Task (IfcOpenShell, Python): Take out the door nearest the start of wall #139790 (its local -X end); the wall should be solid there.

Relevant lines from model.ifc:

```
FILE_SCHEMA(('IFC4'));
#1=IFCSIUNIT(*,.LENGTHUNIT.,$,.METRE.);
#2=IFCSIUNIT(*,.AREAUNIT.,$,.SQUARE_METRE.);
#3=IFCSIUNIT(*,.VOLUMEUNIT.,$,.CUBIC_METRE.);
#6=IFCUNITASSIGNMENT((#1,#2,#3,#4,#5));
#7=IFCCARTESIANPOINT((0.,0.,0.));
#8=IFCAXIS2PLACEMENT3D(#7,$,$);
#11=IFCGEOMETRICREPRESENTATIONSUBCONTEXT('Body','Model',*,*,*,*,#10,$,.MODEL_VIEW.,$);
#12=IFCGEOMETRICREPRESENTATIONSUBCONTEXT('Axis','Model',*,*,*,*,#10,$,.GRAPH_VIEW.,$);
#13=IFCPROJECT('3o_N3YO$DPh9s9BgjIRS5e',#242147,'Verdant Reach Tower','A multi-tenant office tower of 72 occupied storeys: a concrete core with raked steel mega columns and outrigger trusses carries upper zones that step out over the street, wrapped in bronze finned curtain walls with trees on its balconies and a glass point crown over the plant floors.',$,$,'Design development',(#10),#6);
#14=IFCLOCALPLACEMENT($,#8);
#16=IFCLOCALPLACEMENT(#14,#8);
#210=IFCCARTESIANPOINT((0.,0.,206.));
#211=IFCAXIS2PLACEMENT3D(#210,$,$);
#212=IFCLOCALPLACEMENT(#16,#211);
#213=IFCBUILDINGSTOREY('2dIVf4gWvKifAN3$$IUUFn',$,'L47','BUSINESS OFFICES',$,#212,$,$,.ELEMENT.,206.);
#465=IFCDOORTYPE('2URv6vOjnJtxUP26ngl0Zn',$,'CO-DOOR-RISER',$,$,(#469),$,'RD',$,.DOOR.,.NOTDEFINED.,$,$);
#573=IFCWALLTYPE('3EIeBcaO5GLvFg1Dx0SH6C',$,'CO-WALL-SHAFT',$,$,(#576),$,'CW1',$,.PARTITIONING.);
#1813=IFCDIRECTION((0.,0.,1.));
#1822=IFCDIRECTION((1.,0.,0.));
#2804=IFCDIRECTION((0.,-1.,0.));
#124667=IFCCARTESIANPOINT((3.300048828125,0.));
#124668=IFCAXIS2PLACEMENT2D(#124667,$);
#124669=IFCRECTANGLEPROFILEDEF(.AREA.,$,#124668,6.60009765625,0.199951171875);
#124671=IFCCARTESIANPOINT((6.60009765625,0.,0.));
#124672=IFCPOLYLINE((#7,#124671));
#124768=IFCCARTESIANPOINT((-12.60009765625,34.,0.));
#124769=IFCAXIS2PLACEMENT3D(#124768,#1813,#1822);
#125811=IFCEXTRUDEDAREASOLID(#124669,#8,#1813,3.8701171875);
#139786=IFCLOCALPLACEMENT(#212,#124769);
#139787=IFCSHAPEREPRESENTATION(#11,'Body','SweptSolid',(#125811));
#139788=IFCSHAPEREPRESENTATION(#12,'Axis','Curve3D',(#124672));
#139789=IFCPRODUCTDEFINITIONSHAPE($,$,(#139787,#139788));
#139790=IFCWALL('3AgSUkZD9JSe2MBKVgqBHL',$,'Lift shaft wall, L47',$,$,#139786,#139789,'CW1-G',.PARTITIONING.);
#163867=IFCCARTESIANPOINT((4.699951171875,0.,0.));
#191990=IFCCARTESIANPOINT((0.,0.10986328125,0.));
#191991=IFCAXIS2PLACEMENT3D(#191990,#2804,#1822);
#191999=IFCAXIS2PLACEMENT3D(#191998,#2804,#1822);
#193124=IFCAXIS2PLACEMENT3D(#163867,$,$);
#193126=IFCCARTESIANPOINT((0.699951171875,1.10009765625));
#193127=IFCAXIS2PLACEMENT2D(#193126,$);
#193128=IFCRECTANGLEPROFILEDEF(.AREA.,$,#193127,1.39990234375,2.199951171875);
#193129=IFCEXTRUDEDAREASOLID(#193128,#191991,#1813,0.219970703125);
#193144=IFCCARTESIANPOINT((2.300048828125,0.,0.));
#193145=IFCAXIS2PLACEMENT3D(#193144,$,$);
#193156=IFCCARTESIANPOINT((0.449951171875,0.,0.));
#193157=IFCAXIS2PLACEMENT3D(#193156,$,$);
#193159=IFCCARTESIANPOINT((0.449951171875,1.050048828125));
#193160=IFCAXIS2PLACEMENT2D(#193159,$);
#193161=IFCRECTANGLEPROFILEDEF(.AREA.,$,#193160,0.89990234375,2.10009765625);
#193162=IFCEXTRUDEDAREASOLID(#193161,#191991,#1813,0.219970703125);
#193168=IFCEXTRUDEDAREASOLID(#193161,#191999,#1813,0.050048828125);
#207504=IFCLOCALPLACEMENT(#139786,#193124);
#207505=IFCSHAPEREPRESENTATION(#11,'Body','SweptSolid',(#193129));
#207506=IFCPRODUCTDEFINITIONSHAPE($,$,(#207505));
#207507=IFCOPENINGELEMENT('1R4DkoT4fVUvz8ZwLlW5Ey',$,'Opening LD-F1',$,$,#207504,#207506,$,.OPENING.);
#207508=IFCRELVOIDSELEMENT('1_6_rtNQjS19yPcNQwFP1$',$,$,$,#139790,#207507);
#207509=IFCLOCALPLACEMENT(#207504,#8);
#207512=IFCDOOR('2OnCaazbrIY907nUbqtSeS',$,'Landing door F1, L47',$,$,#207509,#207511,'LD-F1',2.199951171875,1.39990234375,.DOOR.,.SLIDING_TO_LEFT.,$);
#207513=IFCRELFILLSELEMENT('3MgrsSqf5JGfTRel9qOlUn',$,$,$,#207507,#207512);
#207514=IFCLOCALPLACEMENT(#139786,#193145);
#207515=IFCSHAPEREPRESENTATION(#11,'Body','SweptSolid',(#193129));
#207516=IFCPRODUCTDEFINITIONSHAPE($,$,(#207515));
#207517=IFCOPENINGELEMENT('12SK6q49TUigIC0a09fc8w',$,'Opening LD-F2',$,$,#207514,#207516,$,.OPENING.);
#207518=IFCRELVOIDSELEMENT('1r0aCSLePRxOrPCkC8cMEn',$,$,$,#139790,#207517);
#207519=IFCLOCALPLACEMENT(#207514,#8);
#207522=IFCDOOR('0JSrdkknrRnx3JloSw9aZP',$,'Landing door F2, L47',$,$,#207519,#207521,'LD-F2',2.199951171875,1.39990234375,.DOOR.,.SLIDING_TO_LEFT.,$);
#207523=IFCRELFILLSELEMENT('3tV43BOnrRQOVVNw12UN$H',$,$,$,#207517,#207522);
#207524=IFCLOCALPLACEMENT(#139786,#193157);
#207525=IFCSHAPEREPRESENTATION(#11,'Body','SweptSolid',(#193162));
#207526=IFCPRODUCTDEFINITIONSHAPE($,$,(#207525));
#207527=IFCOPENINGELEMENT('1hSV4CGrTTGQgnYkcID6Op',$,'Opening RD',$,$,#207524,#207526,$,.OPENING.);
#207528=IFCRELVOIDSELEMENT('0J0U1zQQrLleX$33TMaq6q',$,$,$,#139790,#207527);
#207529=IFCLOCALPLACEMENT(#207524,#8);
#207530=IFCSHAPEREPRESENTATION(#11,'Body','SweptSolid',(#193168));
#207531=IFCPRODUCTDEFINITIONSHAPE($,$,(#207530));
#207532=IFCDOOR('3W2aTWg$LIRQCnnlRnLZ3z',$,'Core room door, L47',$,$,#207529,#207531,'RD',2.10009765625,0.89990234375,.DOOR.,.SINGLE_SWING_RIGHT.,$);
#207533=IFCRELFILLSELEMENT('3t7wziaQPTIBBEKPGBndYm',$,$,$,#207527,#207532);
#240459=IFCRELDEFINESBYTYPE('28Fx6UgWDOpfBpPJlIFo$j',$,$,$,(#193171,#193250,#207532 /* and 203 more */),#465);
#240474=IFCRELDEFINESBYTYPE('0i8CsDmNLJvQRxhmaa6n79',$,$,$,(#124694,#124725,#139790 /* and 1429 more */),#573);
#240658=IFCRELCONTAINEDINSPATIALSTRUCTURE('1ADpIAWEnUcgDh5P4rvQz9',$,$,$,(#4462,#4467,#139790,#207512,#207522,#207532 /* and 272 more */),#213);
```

```python
import ifcopenshell
import ifcopenshell.api.feature
import ifcopenshell.api.root
import ifcopenshell.geom
import ifcopenshell.util.shape

model = ifcopenshell.open("model.ifc")
settings = ifcopenshell.geom.settings()


def volume(element):
    """Net volume in cubic metres, openings subtracted."""
    shape = ifcopenshell.geom.create_shape(settings, element)
    return ifcopenshell.util.shape.get_volume(shape.geometry)


door = model.by_guid("3W2aTWg$LIRQCnnlRnLZ3z")
opening = door.FillsVoids[0].RelatingOpeningElement
wall = opening.VoidsElements[0].RelatingBuildingElement
before = volume(wall)

ifcopenshell.api.root.remove_product(model, product=door)
ifcopenshell.api.feature.remove_feature(model, feature=opening)

after = volume(wall)

print(f"wall volume {before:.3f} -> {after:.3f} m3")

model.write("model-out.ifc")
```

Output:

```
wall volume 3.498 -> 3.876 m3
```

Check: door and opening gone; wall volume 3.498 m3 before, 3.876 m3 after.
